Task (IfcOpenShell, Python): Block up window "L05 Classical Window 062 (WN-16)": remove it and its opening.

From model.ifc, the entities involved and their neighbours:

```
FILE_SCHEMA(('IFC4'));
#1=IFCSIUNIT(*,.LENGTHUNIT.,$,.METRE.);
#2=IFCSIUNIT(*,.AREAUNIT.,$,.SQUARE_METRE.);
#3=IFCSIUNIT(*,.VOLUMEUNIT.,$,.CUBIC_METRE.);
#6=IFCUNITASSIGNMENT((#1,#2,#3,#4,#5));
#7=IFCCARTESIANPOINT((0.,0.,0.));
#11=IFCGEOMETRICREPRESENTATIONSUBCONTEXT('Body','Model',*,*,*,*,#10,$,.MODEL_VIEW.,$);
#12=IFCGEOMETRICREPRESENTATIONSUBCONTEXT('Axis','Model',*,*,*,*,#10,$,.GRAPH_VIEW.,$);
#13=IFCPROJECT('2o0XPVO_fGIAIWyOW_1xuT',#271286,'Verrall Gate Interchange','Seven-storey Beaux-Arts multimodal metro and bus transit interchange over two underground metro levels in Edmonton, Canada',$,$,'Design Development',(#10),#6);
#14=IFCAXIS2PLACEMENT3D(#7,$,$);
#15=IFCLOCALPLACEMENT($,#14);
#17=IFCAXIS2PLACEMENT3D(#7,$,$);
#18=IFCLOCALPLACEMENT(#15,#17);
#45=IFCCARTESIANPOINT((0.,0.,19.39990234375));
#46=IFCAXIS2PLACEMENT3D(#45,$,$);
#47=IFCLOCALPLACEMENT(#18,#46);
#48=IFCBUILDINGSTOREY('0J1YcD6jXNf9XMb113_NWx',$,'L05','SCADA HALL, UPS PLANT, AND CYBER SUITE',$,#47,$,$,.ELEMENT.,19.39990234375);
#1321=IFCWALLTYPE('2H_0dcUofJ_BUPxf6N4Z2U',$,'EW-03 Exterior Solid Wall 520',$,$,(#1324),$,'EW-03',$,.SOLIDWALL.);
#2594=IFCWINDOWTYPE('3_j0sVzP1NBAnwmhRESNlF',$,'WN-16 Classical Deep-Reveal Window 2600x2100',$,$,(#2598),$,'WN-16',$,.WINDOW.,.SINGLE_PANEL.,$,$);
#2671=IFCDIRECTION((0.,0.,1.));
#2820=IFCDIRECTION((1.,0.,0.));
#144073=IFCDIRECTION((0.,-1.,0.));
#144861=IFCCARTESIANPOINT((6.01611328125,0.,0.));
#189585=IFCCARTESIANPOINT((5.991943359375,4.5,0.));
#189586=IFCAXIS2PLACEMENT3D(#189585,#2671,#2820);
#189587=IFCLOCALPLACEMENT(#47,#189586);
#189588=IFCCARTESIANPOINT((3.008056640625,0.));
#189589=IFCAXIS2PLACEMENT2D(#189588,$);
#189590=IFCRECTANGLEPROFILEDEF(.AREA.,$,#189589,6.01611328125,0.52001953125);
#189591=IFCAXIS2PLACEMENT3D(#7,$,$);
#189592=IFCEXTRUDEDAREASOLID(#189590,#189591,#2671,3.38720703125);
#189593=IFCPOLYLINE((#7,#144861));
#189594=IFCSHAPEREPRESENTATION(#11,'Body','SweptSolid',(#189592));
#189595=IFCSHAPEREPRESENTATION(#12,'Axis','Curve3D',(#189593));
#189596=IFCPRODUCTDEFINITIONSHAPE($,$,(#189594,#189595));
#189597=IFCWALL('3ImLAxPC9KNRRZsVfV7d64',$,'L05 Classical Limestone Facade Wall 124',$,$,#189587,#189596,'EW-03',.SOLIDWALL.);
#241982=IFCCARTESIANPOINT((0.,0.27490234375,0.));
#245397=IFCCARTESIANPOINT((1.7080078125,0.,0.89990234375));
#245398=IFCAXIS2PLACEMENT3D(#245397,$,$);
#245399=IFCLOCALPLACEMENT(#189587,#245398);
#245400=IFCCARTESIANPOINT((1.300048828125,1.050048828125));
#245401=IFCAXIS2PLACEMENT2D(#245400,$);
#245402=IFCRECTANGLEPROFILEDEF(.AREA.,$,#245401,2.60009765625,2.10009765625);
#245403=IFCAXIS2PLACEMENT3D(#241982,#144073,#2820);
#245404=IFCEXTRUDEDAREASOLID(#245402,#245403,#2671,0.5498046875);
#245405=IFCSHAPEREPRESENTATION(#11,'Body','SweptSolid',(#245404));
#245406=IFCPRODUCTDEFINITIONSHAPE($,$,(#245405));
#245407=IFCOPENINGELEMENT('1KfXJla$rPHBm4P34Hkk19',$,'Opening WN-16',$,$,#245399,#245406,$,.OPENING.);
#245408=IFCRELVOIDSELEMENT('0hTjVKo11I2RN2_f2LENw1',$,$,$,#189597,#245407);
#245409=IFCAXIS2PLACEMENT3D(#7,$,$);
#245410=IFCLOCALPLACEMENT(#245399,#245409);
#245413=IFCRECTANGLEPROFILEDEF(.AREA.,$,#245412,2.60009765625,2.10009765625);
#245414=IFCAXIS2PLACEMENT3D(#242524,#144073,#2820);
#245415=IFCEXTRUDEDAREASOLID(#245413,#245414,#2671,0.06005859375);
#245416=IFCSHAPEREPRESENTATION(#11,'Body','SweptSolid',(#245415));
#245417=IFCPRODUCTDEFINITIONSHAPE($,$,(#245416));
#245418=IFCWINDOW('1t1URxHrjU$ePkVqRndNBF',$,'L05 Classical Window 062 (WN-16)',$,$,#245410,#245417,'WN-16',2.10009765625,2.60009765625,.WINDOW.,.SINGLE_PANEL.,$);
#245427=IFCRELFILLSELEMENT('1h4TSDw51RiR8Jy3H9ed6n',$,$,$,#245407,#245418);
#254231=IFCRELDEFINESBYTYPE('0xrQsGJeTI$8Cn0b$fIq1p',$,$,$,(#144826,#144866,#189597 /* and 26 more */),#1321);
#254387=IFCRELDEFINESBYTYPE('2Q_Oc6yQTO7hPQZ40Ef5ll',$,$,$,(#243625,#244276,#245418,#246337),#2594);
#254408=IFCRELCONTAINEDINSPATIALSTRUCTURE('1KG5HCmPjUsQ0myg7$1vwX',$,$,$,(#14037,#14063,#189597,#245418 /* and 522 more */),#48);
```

```python
import ifcopenshell
import ifcopenshell.api.feature
import ifcopenshell.api.root
import ifcopenshell.geom
import ifcopenshell.util.shape

model = ifcopenshell.open("model.ifc")
settings = ifcopenshell.geom.settings()


def volume(element):
    """Net volume in cubic metres, openings subtracted."""
    shape = ifcopenshell.geom.create_shape(settings, element)
    return ifcopenshell.util.shape.get_volume(shape.geometry)


window = model.by_guid("1t1URxHrjU$ePkVqRndNBF")
opening = window.FillsVoids[0].RelatingOpeningElement
wall = opening.VoidsElements[0].RelatingBuildingElement
before = volume(wall)

ifcopenshell.api.root.remove_product(model, product=window)
ifcopenshell.api.feature.remove_feature(model, feature=opening)

after = volume(wall)

print(f"wall volume {before:.3f} -> {after:.3f} m3")

model.write("model_updated.ifc")
```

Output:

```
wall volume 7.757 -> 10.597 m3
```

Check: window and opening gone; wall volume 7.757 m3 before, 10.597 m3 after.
